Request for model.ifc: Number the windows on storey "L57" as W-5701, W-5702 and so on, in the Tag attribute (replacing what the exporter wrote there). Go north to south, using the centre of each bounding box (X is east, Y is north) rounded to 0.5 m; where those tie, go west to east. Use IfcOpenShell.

First a look at what the model holds.

```python
import ifcopenshell
import ifcopenshell.util.element
import ifcopenshell.util.placement

model = ifcopenshell.open("model.ifc")
print(model.schema)
storey = next(s for s in model.by_type("IfcBuildingStorey") if s.Name == "L57")
windows = [e for e in ifcopenshell.util.element.get_decomposition(storey) if e.is_a("IfcWindow")]
for e in sorted(windows, key=lambda e: e.id()):
    origin = ifcopenshell.util.placement.get_local_placement(e.ObjectPlacement)[:3, 3]
    print(e.id(), e.Tag, e.Name, origin.round(2) + 0.0, sep=" | ")
```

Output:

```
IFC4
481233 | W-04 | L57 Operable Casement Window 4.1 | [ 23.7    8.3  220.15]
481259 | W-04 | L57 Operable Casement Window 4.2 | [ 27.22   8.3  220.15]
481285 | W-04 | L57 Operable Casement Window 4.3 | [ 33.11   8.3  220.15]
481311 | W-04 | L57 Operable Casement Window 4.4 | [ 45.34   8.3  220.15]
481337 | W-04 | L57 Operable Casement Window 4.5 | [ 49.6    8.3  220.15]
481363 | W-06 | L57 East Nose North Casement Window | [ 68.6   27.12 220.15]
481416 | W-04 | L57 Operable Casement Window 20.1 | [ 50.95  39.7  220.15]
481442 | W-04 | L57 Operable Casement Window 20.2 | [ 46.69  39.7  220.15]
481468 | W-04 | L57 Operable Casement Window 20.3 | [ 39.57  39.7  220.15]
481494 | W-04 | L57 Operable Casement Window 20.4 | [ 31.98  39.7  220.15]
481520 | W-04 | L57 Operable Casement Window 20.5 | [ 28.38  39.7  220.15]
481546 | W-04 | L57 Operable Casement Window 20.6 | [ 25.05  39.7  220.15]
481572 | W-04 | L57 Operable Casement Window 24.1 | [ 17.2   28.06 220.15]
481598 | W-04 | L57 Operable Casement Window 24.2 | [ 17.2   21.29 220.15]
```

```python
import ifcopenshell
import ifcopenshell.geom
import ifcopenshell.util.element
import ifcopenshell.util.shape

model = ifcopenshell.open("model.ifc")
settings = ifcopenshell.geom.settings()
settings.set("use-world-coords", True)


def centre(element):
    shape = ifcopenshell.geom.create_shape(settings, element)
    return ifcopenshell.util.shape.get_bbox_centroid(shape.geometry)


storey = next(s for s in model.by_type("IfcBuildingStorey") if s.Name == "L57")
windows = [e for e in ifcopenshell.util.element.get_decomposition(storey) if e.is_a("IfcWindow")]

# Insertion points can sit at a corner or the storey origin, so sort by the geometry (in metres).
centres = {e: centre(e) for e in windows}
windows.sort(key=lambda e: (-round(centres[e][1] / 0.5), centres[e][0]))

for i, e in enumerate(windows, start=1):
    number = f"W-57{i:02d}"
    e.Tag = number
    print(e.id(), number)

model.write("model-out.ifc")
```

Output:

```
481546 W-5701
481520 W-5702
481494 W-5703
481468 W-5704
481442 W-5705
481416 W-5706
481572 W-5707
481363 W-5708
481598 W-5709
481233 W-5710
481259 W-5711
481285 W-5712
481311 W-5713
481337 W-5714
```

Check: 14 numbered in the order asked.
